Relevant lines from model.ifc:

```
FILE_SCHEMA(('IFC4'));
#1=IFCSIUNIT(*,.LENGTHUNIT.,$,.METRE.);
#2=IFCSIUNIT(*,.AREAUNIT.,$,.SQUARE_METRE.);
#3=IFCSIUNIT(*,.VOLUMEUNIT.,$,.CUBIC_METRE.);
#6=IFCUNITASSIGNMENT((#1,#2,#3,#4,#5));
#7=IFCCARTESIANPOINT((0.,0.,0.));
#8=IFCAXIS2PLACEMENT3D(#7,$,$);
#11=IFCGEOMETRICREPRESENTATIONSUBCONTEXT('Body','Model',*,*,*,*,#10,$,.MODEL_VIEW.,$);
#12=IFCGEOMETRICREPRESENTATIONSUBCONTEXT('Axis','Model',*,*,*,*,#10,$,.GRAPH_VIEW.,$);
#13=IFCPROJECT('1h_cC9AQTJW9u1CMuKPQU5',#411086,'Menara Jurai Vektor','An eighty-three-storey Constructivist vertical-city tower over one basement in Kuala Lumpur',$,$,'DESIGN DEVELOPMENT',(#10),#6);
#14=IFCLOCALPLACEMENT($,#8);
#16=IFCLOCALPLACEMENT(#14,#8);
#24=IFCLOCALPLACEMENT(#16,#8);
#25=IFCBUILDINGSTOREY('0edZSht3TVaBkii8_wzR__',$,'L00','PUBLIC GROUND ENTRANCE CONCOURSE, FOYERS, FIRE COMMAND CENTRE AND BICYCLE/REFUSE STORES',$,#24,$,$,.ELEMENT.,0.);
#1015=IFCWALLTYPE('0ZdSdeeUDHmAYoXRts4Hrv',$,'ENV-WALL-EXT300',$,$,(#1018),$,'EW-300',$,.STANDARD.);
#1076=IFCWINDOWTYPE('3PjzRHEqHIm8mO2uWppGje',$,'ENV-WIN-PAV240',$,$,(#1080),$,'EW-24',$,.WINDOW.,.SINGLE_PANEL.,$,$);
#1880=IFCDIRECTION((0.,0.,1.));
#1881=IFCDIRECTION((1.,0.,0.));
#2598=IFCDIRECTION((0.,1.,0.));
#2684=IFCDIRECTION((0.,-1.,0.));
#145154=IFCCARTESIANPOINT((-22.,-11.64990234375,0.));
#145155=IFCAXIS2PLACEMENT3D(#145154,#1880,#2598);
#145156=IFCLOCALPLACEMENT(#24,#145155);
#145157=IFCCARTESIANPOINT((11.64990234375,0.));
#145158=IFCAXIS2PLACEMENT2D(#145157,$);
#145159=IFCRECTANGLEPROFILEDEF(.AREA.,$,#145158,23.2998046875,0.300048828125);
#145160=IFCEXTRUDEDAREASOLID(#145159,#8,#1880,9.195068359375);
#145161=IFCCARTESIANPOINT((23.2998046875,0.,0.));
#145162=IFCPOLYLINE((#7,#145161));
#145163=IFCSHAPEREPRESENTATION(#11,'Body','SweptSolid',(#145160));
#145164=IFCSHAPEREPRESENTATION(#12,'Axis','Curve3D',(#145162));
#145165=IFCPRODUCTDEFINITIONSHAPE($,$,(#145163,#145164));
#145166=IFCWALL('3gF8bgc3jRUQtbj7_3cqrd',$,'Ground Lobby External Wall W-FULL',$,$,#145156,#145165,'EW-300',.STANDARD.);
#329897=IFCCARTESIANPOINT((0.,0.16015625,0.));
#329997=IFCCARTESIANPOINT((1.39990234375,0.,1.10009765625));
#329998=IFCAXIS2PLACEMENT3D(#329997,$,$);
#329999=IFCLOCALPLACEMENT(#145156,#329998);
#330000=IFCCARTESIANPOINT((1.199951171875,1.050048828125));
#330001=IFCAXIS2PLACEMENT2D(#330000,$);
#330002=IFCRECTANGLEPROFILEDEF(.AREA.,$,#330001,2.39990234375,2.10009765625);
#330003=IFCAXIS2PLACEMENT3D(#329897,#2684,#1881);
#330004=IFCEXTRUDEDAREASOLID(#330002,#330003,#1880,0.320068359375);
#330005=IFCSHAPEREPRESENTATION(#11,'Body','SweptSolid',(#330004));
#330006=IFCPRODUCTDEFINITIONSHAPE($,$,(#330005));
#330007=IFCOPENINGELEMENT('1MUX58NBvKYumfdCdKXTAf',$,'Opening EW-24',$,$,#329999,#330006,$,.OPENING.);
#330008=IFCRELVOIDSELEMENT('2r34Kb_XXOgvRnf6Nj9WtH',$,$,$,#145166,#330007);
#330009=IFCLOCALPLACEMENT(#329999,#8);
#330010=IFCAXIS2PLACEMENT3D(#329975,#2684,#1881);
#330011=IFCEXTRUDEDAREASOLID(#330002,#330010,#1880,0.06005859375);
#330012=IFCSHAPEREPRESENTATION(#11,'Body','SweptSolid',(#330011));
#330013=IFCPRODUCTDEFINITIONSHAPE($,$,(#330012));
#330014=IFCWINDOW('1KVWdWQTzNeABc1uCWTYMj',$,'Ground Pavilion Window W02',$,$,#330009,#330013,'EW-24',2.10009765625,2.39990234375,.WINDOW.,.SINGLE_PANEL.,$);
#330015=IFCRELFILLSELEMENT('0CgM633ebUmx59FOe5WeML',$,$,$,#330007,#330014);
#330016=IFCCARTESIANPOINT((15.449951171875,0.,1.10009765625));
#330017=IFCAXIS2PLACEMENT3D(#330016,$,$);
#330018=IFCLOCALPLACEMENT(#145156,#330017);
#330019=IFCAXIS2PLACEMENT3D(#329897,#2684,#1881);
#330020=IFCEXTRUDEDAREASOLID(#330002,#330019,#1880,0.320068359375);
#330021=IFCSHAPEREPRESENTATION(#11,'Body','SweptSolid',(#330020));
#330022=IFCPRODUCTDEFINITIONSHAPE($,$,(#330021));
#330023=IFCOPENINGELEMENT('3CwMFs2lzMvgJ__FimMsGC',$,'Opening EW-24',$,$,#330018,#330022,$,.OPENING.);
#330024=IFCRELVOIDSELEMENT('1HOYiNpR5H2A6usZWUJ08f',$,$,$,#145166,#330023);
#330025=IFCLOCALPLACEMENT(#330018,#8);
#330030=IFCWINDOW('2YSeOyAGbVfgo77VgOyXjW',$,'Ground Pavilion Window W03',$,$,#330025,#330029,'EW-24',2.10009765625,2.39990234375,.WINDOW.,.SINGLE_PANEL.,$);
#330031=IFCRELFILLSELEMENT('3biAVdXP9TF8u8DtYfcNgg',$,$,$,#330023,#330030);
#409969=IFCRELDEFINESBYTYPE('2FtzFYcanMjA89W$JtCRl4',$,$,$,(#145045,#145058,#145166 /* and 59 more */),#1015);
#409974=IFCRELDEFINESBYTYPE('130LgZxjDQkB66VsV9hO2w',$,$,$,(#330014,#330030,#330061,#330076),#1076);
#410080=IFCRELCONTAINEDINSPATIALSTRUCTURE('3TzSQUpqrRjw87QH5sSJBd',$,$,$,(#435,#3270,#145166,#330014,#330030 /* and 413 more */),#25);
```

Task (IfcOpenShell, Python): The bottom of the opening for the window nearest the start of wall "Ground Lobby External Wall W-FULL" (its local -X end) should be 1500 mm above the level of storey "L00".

```python
import numpy as np
import ifcopenshell
import ifcopenshell.api.geometry
import ifcopenshell.geom
import ifcopenshell.util.element
import ifcopenshell.util.placement
import ifcopenshell.util.shape
import ifcopenshell.util.unit

model = ifcopenshell.open("model.ifc")
unit_scale = ifcopenshell.util.unit.calculate_unit_scale(model)

window = model.by_guid("1KVWdWQTzNeABc1uCWTYMj")
opening = window.FillsVoids[0].RelatingOpeningElement
storey = ifcopenshell.util.element.get_container(window, ifc_class="IfcBuildingStorey")
level = ifcopenshell.util.placement.get_local_placement(storey.ObjectPlacement)[2, 3]

# The opening's origin need not be at the sill, so measure its lowest point.
shape = ifcopenshell.geom.create_shape(ifcopenshell.geom.settings(), opening)
bottom = ifcopenshell.util.shape.get_shape_bottom_elevation(shape, shape.geometry) / unit_scale
dz = level + 1.5 - bottom

shift = np.array([0.0, 0.0, dz])
# The window is placed relative to its opening, so it follows when the opening moves.
matrix = ifcopenshell.util.placement.get_local_placement(opening.ObjectPlacement)
matrix[:3, 3] += shift
ifcopenshell.api.geometry.edit_object_placement(
    model, product=opening, matrix=matrix, is_si=False, should_transform_children=True
)

print(f"moved by {dz * unit_scale:+.3f} m")

model.write("model_updated.ifc")
```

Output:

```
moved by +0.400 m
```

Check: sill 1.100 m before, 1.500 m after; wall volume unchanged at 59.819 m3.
